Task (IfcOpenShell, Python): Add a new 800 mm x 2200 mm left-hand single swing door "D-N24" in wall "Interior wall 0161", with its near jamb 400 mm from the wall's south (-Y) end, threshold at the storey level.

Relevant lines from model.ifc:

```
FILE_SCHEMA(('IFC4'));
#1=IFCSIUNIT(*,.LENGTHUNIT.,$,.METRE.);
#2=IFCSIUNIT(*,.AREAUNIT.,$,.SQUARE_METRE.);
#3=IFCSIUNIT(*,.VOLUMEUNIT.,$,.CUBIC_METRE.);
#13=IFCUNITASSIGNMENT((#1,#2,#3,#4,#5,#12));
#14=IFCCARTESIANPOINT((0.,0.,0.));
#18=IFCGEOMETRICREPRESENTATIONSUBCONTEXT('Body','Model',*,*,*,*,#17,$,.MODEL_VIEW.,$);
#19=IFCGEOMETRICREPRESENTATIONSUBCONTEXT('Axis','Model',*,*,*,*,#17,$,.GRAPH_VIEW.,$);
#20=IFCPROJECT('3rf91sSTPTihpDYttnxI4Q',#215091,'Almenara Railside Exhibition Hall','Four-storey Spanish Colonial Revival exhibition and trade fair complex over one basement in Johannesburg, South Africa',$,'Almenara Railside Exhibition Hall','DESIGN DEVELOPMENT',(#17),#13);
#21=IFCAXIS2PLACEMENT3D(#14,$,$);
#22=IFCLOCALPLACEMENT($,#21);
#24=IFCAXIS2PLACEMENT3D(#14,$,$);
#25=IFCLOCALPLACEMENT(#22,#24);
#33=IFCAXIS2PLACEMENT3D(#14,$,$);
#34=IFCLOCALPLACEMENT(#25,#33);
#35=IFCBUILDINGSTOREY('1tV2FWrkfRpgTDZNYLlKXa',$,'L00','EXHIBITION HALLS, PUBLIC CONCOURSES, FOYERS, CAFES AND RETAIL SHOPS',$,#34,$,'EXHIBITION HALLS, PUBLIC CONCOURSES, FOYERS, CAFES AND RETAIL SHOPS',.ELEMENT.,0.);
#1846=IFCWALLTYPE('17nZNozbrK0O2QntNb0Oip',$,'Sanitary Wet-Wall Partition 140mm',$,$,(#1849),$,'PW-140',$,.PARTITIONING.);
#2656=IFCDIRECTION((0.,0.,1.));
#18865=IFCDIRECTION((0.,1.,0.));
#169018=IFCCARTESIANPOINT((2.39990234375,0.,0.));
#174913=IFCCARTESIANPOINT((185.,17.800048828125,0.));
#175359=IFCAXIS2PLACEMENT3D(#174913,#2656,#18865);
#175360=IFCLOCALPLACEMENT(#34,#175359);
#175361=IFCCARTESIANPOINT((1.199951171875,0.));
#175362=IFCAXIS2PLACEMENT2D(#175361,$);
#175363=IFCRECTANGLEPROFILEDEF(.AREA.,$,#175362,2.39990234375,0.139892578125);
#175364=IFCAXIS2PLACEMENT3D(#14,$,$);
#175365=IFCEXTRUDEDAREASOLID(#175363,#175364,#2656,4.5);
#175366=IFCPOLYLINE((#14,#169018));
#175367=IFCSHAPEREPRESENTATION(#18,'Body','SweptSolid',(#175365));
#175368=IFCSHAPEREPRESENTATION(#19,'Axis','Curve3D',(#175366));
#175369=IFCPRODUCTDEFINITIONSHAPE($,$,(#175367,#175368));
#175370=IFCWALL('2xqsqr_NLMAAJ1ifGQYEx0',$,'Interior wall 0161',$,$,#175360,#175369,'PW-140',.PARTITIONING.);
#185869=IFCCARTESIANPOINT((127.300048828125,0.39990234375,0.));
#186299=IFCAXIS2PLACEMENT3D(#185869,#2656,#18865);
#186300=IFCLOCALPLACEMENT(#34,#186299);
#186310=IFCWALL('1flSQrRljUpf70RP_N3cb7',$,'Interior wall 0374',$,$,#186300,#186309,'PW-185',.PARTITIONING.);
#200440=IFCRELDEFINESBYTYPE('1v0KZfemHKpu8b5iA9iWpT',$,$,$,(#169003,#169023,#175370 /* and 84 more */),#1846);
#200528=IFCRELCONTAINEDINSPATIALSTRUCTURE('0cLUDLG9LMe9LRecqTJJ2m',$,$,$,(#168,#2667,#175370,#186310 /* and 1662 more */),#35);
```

```python
import numpy as np
import ifcopenshell
import ifcopenshell.api.feature
import ifcopenshell.api.geometry
import ifcopenshell.api.root
import ifcopenshell.api.spatial
import ifcopenshell.geom
import ifcopenshell.util.element
import ifcopenshell.util.placement
import ifcopenshell.util.representation
import ifcopenshell.util.shape
import ifcopenshell.util.unit

model = ifcopenshell.open("model.ifc")
unit_scale = ifcopenshell.util.unit.calculate_unit_scale(model)
settings = ifcopenshell.geom.settings()


def volume(element):
    """Net volume in cubic metres, openings subtracted."""
    shape = ifcopenshell.geom.create_shape(settings, element)
    return ifcopenshell.util.shape.get_volume(shape.geometry)


wall = model.by_guid("2xqsqr_NLMAAJ1ifGQYEx0")
storey = ifcopenshell.util.element.get_container(wall, ifc_class="IfcBuildingStorey")
context = ifcopenshell.util.representation.get_context(model, "Model", "Body", "MODEL_VIEW")
before = volume(wall)

width, height, from_end, sill = 0.8, 2.2, 0.4, 0.0  # metres

# The wall runs along its own X axis, and the end named is its -X end.
wall_shape = ifcopenshell.geom.create_shape(settings, wall)
x, y, z = ifcopenshell.util.shape.get_vertices(wall_shape.geometry).T
start = x.min() + from_end
face, thickness = float(y.min()), float(y.max() - y.min())
wall_matrix = ifcopenshell.util.placement.get_local_placement(wall.ObjectPlacement)
level = ifcopenshell.util.placement.get_local_placement(storey.ObjectPlacement)[2, 3]


def in_wall(x, y):
    """Placement at x, y metres in the wall's axes, at sill height."""
    matrix = wall_matrix.copy()
    matrix[:, 3] = wall_matrix @ np.array([x / unit_scale, y / unit_scale, 0.0, 1.0])
    matrix[2, 3] = level + sill / unit_scale
    return matrix


# Opening: a box that overshoots both wall faces by 50 mm.
opening = ifcopenshell.api.root.create_entity(model, ifc_class="IfcOpeningElement", predefined_type="OPENING")
box = ifcopenshell.api.geometry.add_wall_representation(
    model, context=context, length=width, height=height, thickness=thickness + 0.1
)
ifcopenshell.api.geometry.assign_representation(model, product=opening, representation=box)
ifcopenshell.api.geometry.edit_object_placement(model, product=opening, matrix=in_wall(start, face - 0.05), is_si=False)
ifcopenshell.api.feature.add_feature(model, feature=opening, element=wall)

door = ifcopenshell.api.root.create_entity(model, ifc_class="IfcDoor", name="D-N24", predefined_type="DOOR")
door.OverallWidth, door.OverallHeight = width / unit_scale, height / unit_scale
door.OperationType = "SINGLE_SWING_LEFT"
body = ifcopenshell.api.geometry.add_door_representation(
    model,
    context=context,
    overall_width=door.OverallWidth,
    overall_height=door.OverallHeight,
    operation_type="SINGLE_SWING_LEFT",
    lining_properties={"LiningDepth": thickness / unit_scale, "ThresholdDepth": thickness / unit_scale},
)
ifcopenshell.api.geometry.assign_representation(model, product=door, representation=body)
ifcopenshell.api.spatial.assign_container(model, products=[door], relating_structure=storey)
ifcopenshell.api.feature.add_filling(model, opening=opening, element=door)

# The lining spans the wall, so the door starts at the wall face.
ifcopenshell.api.geometry.edit_object_placement(model, product=door, matrix=in_wall(start, face), is_si=False)

after = volume(wall)

print(f"wall volume {before:.3f} -> {after:.3f} m3")

model.write("model-out.ifc")
```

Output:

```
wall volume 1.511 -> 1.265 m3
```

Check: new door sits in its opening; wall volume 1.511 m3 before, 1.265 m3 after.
